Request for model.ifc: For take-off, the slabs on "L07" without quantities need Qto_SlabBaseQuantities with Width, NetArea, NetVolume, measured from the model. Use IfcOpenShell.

First a look at what the model holds.

```python
import ifcopenshell
import ifcopenshell.util.element
import ifcopenshell.util.unit

model = ifcopenshell.open("model.ifc")
print(model.schema)
for unit_type in ("LENGTHUNIT", "AREAUNIT", "VOLUMEUNIT"):
    print(unit_type, ifcopenshell.util.unit.calculate_unit_scale(model, unit_type))
storey = next(s for s in model.by_type("IfcBuildingStorey") if s.Name == "L07")
slabs = [e for e in ifcopenshell.util.element.get_decomposition(storey) if e.is_a("IfcSlab")]
for e in sorted(slabs, key=lambda e: e.id()):
    print(e.id(), e.is_a(), e.Name, list(ifcopenshell.util.element.get_psets(e, qtos_only=True)), sep=" | ")
```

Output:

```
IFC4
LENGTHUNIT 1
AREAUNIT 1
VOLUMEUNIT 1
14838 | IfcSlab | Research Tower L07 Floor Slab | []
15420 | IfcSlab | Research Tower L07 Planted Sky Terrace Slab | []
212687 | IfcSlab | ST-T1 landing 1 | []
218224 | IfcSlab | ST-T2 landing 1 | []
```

```python
import ifcopenshell
import ifcopenshell.api.pset
import ifcopenshell.geom
import ifcopenshell.util.element
import ifcopenshell.util.shape
import ifcopenshell.util.unit

model = ifcopenshell.open("model.ifc")
unit_scale = ifcopenshell.util.unit.calculate_unit_scale(model)
area_scale = ifcopenshell.util.unit.calculate_unit_scale(model, "AREAUNIT")
volume_scale = ifcopenshell.util.unit.calculate_unit_scale(model, "VOLUMEUNIT")
settings = ifcopenshell.geom.settings()

storey = next(s for s in model.by_type("IfcBuildingStorey") if s.Name == "L07")
slabs = [e for e in ifcopenshell.util.element.get_decomposition(storey) if e.is_a("IfcSlab")]

for e in sorted(slabs, key=lambda e: e.id()):
    if ifcopenshell.util.element.get_psets(e, qtos_only=True, should_inherit=False):
        continue
    # Geometry comes back in metres, in the element's own axes.
    shape = ifcopenshell.geom.create_shape(settings, e)
    values = {
        "Width": ifcopenshell.util.shape.get_z(shape.geometry) / unit_scale,
        "NetArea": ifcopenshell.util.shape.get_footprint_area(shape.geometry) / area_scale,
        "NetVolume": ifcopenshell.util.shape.get_volume(shape.geometry) / volume_scale,
    }
    qto = ifcopenshell.api.pset.add_qto(model, product=e, name="Qto_SlabBaseQuantities")
    ifcopenshell.api.pset.edit_qto(model, qto=qto, properties=values)
    print(e.id(), {k: round(v, 3) for k, v in values.items()})

model.write("model-out.ifc")
```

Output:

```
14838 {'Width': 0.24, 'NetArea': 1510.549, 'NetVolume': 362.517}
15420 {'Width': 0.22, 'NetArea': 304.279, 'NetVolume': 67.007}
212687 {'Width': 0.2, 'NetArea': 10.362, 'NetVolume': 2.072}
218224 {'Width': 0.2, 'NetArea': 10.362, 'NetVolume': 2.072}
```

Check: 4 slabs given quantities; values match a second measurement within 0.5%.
